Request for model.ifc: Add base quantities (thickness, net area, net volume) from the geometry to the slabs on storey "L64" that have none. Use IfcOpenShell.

First a look at what the model holds.

```python
import ifcopenshell
import ifcopenshell.util.element
import ifcopenshell.util.unit

model = ifcopenshell.open("model.ifc")
print(model.schema)
for unit_type in ("LENGTHUNIT", "AREAUNIT", "VOLUMEUNIT"):
    print(unit_type, ifcopenshell.util.unit.calculate_unit_scale(model, unit_type))
storey = next(s for s in model.by_type("IfcBuildingStorey") if s.Name == "L64")
slabs = [e for e in ifcopenshell.util.element.get_decomposition(storey) if e.is_a("IfcSlab")]
for e in sorted(slabs, key=lambda e: e.id()):
    print(e.id(), e.is_a(), e.Name, list(ifcopenshell.util.element.get_psets(e, qtos_only=True)), sep=" | ")
```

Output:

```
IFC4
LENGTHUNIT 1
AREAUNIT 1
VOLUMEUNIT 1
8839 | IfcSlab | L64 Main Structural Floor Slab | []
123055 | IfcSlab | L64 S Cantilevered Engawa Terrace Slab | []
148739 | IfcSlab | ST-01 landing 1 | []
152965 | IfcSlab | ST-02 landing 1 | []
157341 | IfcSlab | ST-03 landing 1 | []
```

```python
import ifcopenshell
import ifcopenshell.api.pset
import ifcopenshell.geom
import ifcopenshell.util.element
import ifcopenshell.util.shape
import ifcopenshell.util.unit

model = ifcopenshell.open("model.ifc")
unit_scale = ifcopenshell.util.unit.calculate_unit_scale(model)
area_scale = ifcopenshell.util.unit.calculate_unit_scale(model, "AREAUNIT")
volume_scale = ifcopenshell.util.unit.calculate_unit_scale(model, "VOLUMEUNIT")
settings = ifcopenshell.geom.settings()

storey = next(s for s in model.by_type("IfcBuildingStorey") if s.Name == "L64")
slabs = [e for e in ifcopenshell.util.element.get_decomposition(storey) if e.is_a("IfcSlab")]

for e in sorted(slabs, key=lambda e: e.id()):
    if ifcopenshell.util.element.get_psets(e, qtos_only=True, should_inherit=False):
        continue
    # Geometry comes back in metres, in the element's own axes.
    shape = ifcopenshell.geom.create_shape(settings, e)
    values = {
        "Width": ifcopenshell.util.shape.get_z(shape.geometry) / unit_scale,
        "NetArea": ifcopenshell.util.shape.get_footprint_area(shape.geometry) / area_scale,
        "NetVolume": ifcopenshell.util.shape.get_volume(shape.geometry) / volume_scale,
    }
    qto = ifcopenshell.api.pset.add_qto(model, product=e, name="Qto_SlabBaseQuantities")
    ifcopenshell.api.pset.edit_qto(model, qto=qto, properties=values)
    print(e.id(), {k: round(v, 3) for k, v in values.items()})

model.write("model-out.ifc")
```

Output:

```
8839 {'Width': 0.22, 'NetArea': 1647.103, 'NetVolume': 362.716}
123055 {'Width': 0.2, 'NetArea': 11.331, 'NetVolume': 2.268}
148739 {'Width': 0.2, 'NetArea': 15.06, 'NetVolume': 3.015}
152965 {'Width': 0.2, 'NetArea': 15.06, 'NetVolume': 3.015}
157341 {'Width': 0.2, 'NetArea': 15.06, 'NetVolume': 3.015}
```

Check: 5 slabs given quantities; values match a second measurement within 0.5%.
